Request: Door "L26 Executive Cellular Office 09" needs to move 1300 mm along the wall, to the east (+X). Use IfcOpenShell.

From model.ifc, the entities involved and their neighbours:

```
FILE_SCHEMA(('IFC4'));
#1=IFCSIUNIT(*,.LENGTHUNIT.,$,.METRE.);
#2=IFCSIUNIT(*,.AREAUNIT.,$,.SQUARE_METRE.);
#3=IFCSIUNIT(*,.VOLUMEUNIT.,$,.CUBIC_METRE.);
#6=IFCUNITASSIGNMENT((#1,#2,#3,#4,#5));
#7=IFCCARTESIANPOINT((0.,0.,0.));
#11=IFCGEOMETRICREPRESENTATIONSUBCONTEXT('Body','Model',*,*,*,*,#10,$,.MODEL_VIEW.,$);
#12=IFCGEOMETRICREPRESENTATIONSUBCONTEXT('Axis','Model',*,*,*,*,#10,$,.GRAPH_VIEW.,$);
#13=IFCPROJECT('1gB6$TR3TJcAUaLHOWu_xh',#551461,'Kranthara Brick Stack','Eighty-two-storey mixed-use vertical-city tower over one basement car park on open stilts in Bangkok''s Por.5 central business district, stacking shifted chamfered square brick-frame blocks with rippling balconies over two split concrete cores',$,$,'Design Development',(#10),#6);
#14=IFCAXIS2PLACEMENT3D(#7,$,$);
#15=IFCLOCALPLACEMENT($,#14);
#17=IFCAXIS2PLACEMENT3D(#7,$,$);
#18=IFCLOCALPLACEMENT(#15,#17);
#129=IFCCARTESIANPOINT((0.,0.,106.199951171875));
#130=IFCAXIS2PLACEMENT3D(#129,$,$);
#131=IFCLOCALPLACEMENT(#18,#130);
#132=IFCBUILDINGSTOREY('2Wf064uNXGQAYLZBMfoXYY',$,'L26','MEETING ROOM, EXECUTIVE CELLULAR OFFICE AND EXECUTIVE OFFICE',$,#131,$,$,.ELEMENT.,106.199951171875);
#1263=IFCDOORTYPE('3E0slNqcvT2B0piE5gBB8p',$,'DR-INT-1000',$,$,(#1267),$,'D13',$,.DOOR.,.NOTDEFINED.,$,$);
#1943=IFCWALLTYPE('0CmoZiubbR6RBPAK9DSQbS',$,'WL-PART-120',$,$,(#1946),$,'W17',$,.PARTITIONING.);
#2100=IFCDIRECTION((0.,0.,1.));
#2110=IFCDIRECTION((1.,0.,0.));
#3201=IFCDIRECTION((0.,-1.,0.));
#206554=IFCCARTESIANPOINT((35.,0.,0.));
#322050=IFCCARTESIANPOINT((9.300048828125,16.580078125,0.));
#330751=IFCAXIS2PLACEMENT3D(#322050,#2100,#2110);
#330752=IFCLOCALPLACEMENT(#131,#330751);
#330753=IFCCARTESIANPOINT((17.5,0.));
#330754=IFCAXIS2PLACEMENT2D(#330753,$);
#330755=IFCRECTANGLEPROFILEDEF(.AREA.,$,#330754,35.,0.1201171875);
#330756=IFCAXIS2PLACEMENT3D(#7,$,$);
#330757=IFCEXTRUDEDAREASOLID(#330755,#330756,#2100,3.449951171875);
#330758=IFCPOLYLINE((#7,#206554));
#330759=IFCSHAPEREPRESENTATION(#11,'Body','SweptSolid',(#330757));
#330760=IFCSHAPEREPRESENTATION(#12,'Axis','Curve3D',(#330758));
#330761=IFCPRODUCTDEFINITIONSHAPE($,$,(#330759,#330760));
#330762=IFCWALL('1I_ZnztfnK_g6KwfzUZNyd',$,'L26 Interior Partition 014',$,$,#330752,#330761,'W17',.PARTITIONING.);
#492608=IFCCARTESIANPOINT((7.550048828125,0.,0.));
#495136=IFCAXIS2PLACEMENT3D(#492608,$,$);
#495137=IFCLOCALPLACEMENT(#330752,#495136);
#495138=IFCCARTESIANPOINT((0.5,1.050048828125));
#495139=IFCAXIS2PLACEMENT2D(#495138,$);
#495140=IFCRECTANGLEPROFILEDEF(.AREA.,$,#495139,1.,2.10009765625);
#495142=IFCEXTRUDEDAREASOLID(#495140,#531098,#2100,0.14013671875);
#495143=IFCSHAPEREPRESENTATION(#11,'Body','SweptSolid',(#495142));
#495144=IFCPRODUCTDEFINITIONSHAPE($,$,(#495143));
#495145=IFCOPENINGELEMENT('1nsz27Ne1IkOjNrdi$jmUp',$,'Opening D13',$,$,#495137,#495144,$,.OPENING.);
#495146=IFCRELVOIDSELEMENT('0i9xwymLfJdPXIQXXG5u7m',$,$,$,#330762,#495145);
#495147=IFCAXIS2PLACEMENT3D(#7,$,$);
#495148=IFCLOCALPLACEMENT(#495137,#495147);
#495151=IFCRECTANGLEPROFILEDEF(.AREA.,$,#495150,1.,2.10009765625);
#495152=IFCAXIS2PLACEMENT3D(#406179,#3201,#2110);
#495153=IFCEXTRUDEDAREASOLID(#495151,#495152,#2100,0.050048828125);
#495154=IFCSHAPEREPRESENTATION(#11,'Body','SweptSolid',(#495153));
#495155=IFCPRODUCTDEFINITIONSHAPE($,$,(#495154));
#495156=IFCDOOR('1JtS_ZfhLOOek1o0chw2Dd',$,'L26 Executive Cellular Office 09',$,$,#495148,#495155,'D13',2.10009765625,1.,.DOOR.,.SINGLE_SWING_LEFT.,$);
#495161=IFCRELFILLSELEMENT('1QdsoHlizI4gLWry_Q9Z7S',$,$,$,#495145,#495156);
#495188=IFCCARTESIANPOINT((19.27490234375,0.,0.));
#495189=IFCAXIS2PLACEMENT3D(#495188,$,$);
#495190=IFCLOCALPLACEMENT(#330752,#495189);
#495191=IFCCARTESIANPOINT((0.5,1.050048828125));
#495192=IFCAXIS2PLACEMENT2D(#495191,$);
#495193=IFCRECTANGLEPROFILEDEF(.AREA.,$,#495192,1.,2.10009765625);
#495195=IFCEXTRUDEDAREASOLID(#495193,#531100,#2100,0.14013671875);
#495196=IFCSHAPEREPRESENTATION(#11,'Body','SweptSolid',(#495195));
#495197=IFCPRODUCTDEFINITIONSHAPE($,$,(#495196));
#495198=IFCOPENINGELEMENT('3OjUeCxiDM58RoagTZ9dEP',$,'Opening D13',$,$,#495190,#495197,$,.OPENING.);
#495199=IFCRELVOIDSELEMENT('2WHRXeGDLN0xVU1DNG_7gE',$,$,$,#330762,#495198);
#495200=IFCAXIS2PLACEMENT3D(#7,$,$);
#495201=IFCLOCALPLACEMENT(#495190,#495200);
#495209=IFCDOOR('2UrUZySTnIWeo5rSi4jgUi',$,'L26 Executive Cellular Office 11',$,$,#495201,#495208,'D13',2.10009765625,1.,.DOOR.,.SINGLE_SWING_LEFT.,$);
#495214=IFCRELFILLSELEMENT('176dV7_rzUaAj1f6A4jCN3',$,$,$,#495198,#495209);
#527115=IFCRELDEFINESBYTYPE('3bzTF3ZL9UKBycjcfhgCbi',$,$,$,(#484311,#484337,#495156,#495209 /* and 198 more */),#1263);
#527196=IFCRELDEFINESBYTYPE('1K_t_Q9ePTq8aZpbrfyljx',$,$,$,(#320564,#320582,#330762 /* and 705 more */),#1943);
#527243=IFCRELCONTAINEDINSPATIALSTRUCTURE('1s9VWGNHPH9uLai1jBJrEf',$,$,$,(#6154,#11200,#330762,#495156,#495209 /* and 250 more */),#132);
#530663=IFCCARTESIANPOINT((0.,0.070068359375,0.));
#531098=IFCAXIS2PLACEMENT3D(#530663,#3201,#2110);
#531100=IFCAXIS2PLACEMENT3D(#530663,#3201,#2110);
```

```python
import ifcopenshell
import ifcopenshell.api.geometry
import ifcopenshell.util.placement
import ifcopenshell.util.unit

model = ifcopenshell.open("model.ifc")
unit_scale = ifcopenshell.util.unit.calculate_unit_scale(model)

door = model.by_guid("1JtS_ZfhLOOek1o0chw2Dd")
opening = door.FillsVoids[0].RelatingOpeningElement
wall = opening.VoidsElements[0].RelatingBuildingElement

wall_matrix = ifcopenshell.util.placement.get_local_placement(wall.ObjectPlacement)
shift = wall_matrix[:3, 0] * 1.3 / unit_scale
before = ifcopenshell.util.placement.get_local_placement(door.ObjectPlacement)[:3, 3].copy()

# The door is placed relative to its opening, so it follows when the opening moves.
matrix = ifcopenshell.util.placement.get_local_placement(opening.ObjectPlacement)
matrix[:3, 3] += shift
ifcopenshell.api.geometry.edit_object_placement(
    model, product=opening, matrix=matrix, is_si=False, should_transform_children=True
)

after = ifcopenshell.util.placement.get_local_placement(door.ObjectPlacement)[:3, 3]
print("door moved by", (after - before).round(3) + 0.0)

model.write("model_v2.ifc")
```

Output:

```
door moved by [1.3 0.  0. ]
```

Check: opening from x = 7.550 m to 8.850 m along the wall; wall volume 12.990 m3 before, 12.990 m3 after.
